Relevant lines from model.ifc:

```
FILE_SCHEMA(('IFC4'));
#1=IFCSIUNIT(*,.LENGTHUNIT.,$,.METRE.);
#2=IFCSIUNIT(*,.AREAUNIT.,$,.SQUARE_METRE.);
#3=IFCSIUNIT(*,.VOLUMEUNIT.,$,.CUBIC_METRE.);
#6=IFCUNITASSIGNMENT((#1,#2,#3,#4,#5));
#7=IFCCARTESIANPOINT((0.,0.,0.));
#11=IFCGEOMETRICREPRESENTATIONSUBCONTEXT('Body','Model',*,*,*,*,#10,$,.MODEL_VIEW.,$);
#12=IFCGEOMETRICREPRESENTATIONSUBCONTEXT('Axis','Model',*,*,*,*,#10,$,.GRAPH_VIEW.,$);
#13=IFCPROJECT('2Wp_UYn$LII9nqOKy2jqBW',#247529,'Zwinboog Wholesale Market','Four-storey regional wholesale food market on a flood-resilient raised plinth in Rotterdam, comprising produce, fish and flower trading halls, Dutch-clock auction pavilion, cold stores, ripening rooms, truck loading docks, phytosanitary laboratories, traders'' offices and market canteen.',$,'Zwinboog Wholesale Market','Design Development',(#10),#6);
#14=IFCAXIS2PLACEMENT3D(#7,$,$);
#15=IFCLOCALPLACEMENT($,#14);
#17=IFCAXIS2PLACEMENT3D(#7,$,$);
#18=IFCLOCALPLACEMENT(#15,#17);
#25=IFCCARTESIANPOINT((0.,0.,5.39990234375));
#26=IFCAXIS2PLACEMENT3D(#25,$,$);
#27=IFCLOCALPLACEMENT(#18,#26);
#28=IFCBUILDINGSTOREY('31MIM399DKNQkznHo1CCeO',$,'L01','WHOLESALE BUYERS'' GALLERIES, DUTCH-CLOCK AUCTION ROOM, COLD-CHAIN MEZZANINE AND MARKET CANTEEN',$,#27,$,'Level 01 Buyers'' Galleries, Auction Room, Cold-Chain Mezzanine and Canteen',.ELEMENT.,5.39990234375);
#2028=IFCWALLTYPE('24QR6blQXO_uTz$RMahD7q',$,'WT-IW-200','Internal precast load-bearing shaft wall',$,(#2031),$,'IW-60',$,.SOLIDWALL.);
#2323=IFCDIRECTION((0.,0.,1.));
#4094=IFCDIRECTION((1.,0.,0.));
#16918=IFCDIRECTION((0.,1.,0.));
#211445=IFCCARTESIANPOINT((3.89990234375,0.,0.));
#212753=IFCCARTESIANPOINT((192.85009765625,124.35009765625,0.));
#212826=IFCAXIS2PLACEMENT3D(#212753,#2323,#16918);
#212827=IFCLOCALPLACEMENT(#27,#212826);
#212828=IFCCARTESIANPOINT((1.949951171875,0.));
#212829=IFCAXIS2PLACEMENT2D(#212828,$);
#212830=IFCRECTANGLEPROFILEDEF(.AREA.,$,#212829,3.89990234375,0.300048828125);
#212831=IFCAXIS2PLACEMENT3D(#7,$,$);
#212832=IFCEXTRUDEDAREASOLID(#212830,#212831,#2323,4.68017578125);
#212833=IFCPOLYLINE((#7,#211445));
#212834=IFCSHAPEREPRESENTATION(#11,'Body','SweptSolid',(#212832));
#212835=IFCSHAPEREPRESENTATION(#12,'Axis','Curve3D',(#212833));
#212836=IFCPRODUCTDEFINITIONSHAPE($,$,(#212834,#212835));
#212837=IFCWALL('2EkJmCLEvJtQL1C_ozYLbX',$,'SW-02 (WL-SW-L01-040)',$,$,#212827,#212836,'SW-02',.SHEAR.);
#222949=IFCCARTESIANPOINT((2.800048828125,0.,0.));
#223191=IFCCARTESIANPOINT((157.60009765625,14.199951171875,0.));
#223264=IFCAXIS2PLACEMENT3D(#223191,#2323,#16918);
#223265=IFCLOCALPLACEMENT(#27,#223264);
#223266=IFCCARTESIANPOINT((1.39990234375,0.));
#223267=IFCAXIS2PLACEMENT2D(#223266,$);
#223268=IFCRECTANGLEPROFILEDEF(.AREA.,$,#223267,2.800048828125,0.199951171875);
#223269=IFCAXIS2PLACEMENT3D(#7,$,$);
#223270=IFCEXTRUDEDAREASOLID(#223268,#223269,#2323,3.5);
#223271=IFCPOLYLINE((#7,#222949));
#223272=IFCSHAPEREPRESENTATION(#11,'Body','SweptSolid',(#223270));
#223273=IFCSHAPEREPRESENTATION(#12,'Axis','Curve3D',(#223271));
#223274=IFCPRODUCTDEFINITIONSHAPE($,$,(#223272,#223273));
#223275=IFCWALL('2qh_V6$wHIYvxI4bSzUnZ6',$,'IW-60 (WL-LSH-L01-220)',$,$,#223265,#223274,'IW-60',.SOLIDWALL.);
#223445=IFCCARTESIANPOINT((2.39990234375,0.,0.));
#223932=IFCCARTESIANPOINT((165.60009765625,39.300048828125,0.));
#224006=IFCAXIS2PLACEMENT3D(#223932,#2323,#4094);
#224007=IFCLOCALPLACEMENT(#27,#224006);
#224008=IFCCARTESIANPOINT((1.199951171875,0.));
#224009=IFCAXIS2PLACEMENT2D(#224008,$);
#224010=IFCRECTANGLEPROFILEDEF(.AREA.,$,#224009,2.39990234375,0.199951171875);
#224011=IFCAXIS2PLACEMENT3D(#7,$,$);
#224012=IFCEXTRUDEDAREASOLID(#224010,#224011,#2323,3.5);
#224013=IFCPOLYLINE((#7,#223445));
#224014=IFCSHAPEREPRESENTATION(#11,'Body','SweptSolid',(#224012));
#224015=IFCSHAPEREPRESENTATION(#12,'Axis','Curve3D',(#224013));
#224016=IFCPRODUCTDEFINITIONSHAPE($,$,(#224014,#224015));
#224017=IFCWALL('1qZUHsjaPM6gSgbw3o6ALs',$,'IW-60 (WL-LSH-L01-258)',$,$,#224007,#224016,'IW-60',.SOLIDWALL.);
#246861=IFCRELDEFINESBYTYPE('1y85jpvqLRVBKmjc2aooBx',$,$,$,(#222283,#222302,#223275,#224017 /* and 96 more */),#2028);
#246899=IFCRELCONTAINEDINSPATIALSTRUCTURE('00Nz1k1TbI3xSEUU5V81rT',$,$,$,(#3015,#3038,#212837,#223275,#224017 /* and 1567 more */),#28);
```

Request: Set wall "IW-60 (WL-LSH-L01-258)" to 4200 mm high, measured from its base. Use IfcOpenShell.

```python
import ifcopenshell
import ifcopenshell.geom
import ifcopenshell.util.representation
import ifcopenshell.util.shape
import ifcopenshell.util.unit

model = ifcopenshell.open("model.ifc")
unit_scale = ifcopenshell.util.unit.calculate_unit_scale(model)
settings = ifcopenshell.geom.settings()


def volume(element):
    """Net volume in cubic metres, openings subtracted."""
    shape = ifcopenshell.geom.create_shape(settings, element)
    return ifcopenshell.util.shape.get_volume(shape.geometry)


wall = model.by_id(224017)
before = volume(wall)

body = ifcopenshell.util.representation.get_representation(wall, "Model", "Body")
solid = body.Items[0]
old_height = solid.Depth
solid.Depth = 4.2 / unit_scale
after = volume(wall)

print(f"height {old_height:g} -> {solid.Depth:g}, volume {before:.3f} -> {after:.3f} m3")

model.write("model_edited.ifc")
```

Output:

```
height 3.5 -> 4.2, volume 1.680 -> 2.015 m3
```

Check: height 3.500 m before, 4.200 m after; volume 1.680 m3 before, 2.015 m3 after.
